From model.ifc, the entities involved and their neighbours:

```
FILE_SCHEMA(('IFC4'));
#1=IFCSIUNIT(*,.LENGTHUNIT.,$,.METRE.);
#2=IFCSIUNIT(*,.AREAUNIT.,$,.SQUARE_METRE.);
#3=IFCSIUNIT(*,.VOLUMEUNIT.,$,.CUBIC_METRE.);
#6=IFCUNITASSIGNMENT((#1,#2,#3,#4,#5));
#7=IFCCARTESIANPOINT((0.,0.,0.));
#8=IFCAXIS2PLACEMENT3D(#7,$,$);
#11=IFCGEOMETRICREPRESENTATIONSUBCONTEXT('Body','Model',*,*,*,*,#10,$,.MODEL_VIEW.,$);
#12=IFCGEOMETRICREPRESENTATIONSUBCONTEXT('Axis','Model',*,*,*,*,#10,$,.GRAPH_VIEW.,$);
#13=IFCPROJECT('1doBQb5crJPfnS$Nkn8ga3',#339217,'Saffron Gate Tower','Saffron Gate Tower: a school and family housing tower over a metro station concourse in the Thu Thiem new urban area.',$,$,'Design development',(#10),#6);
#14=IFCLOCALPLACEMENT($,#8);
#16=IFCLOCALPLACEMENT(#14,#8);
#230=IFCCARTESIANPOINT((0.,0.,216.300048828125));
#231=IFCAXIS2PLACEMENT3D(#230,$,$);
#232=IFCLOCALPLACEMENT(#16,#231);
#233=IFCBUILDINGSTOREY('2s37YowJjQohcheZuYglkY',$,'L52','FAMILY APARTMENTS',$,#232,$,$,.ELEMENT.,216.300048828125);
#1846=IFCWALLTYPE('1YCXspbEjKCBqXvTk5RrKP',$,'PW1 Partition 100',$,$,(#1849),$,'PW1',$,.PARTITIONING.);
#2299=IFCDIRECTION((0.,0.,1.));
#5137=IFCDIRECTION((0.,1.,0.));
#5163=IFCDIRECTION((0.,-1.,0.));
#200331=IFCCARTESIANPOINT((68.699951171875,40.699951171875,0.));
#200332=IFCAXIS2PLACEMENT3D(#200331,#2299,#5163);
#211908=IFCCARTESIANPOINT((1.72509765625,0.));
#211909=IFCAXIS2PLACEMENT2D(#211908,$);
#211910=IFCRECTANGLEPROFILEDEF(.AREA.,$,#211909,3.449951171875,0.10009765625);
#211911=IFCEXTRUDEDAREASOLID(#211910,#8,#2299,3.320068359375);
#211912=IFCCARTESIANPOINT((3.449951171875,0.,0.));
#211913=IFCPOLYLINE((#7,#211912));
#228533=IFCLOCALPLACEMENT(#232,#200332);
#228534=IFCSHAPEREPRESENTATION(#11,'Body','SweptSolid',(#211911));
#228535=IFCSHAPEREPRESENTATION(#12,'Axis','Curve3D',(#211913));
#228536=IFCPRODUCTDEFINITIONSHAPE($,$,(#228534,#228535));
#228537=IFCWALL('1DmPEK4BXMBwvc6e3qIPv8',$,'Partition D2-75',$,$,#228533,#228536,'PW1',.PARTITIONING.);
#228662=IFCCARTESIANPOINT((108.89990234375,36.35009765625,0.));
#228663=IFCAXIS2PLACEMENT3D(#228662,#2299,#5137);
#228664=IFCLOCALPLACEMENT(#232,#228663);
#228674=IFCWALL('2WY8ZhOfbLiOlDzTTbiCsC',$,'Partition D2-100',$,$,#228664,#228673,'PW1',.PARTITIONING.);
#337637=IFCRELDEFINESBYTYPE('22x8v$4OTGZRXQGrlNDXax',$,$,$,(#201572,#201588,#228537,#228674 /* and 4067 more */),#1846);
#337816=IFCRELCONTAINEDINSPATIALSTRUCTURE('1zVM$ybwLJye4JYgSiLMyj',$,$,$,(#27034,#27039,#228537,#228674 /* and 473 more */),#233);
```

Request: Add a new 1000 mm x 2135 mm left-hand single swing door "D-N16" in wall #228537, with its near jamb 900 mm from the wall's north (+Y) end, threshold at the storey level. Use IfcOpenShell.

```python
import numpy as np
import ifcopenshell
import ifcopenshell.api.feature
import ifcopenshell.api.geometry
import ifcopenshell.api.root
import ifcopenshell.api.spatial
import ifcopenshell.geom
import ifcopenshell.util.element
import ifcopenshell.util.placement
import ifcopenshell.util.representation
import ifcopenshell.util.shape
import ifcopenshell.util.unit

model = ifcopenshell.open("model.ifc")
unit_scale = ifcopenshell.util.unit.calculate_unit_scale(model)
settings = ifcopenshell.geom.settings()


def volume(element):
    """Net volume in cubic metres, openings subtracted."""
    shape = ifcopenshell.geom.create_shape(settings, element)
    return ifcopenshell.util.shape.get_volume(shape.geometry)


wall = model.by_guid("1DmPEK4BXMBwvc6e3qIPv8")
storey = ifcopenshell.util.element.get_container(wall, ifc_class="IfcBuildingStorey")
context = ifcopenshell.util.representation.get_context(model, "Model", "Body", "MODEL_VIEW")
before = volume(wall)

width, height, from_end, sill = 1, 2.135, 0.9, 0.0  # metres

# The wall runs along its own X axis, and the end named is its -X end.
wall_shape = ifcopenshell.geom.create_shape(settings, wall)
x, y, z = ifcopenshell.util.shape.get_vertices(wall_shape.geometry).T
start = x.min() + from_end
face, thickness = float(y.min()), float(y.max() - y.min())
wall_matrix = ifcopenshell.util.placement.get_local_placement(wall.ObjectPlacement)
level = ifcopenshell.util.placement.get_local_placement(storey.ObjectPlacement)[2, 3]


def in_wall(x, y):
    """Placement at x, y metres in the wall's axes, at sill height."""
    matrix = wall_matrix.copy()
    matrix[:, 3] = wall_matrix @ np.array([x / unit_scale, y / unit_scale, 0.0, 1.0])
    matrix[2, 3] = level + sill / unit_scale
    return matrix


# Opening: a box that overshoots both wall faces by 50 mm.
opening = ifcopenshell.api.root.create_entity(model, ifc_class="IfcOpeningElement", predefined_type="OPENING")
box = ifcopenshell.api.geometry.add_wall_representation(
    model, context=context, length=width, height=height, thickness=thickness + 0.1
)
ifcopenshell.api.geometry.assign_representation(model, product=opening, representation=box)
ifcopenshell.api.geometry.edit_object_placement(model, product=opening, matrix=in_wall(start, face - 0.05), is_si=False)
ifcopenshell.api.feature.add_feature(model, feature=opening, element=wall)

door = ifcopenshell.api.root.create_entity(model, ifc_class="IfcDoor", name="D-N16", predefined_type="DOOR")
door.OverallWidth, door.OverallHeight = width / unit_scale, height / unit_scale
door.OperationType = "SINGLE_SWING_LEFT"
body = ifcopenshell.api.geometry.add_door_representation(
    model,
    context=context,
    overall_width=door.OverallWidth,
    overall_height=door.OverallHeight,
    operation_type="SINGLE_SWING_LEFT",
    lining_properties={"LiningDepth": thickness / unit_scale, "ThresholdDepth": thickness / unit_scale},
)
ifcopenshell.api.geometry.assign_representation(model, product=door, representation=body)
ifcopenshell.api.spatial.assign_container(model, products=[door], relating_structure=storey)
ifcopenshell.api.feature.add_filling(model, opening=opening, element=door)

# The lining spans the wall, so the door starts at the wall face.
ifcopenshell.api.geometry.edit_object_placement(model, product=door, matrix=in_wall(start, face), is_si=False)

after = volume(wall)

print(f"wall volume {before:.3f} -> {after:.3f} m3")

model.write("model_rev.ifc")
```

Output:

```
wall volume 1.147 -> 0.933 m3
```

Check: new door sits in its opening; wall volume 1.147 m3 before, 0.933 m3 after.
